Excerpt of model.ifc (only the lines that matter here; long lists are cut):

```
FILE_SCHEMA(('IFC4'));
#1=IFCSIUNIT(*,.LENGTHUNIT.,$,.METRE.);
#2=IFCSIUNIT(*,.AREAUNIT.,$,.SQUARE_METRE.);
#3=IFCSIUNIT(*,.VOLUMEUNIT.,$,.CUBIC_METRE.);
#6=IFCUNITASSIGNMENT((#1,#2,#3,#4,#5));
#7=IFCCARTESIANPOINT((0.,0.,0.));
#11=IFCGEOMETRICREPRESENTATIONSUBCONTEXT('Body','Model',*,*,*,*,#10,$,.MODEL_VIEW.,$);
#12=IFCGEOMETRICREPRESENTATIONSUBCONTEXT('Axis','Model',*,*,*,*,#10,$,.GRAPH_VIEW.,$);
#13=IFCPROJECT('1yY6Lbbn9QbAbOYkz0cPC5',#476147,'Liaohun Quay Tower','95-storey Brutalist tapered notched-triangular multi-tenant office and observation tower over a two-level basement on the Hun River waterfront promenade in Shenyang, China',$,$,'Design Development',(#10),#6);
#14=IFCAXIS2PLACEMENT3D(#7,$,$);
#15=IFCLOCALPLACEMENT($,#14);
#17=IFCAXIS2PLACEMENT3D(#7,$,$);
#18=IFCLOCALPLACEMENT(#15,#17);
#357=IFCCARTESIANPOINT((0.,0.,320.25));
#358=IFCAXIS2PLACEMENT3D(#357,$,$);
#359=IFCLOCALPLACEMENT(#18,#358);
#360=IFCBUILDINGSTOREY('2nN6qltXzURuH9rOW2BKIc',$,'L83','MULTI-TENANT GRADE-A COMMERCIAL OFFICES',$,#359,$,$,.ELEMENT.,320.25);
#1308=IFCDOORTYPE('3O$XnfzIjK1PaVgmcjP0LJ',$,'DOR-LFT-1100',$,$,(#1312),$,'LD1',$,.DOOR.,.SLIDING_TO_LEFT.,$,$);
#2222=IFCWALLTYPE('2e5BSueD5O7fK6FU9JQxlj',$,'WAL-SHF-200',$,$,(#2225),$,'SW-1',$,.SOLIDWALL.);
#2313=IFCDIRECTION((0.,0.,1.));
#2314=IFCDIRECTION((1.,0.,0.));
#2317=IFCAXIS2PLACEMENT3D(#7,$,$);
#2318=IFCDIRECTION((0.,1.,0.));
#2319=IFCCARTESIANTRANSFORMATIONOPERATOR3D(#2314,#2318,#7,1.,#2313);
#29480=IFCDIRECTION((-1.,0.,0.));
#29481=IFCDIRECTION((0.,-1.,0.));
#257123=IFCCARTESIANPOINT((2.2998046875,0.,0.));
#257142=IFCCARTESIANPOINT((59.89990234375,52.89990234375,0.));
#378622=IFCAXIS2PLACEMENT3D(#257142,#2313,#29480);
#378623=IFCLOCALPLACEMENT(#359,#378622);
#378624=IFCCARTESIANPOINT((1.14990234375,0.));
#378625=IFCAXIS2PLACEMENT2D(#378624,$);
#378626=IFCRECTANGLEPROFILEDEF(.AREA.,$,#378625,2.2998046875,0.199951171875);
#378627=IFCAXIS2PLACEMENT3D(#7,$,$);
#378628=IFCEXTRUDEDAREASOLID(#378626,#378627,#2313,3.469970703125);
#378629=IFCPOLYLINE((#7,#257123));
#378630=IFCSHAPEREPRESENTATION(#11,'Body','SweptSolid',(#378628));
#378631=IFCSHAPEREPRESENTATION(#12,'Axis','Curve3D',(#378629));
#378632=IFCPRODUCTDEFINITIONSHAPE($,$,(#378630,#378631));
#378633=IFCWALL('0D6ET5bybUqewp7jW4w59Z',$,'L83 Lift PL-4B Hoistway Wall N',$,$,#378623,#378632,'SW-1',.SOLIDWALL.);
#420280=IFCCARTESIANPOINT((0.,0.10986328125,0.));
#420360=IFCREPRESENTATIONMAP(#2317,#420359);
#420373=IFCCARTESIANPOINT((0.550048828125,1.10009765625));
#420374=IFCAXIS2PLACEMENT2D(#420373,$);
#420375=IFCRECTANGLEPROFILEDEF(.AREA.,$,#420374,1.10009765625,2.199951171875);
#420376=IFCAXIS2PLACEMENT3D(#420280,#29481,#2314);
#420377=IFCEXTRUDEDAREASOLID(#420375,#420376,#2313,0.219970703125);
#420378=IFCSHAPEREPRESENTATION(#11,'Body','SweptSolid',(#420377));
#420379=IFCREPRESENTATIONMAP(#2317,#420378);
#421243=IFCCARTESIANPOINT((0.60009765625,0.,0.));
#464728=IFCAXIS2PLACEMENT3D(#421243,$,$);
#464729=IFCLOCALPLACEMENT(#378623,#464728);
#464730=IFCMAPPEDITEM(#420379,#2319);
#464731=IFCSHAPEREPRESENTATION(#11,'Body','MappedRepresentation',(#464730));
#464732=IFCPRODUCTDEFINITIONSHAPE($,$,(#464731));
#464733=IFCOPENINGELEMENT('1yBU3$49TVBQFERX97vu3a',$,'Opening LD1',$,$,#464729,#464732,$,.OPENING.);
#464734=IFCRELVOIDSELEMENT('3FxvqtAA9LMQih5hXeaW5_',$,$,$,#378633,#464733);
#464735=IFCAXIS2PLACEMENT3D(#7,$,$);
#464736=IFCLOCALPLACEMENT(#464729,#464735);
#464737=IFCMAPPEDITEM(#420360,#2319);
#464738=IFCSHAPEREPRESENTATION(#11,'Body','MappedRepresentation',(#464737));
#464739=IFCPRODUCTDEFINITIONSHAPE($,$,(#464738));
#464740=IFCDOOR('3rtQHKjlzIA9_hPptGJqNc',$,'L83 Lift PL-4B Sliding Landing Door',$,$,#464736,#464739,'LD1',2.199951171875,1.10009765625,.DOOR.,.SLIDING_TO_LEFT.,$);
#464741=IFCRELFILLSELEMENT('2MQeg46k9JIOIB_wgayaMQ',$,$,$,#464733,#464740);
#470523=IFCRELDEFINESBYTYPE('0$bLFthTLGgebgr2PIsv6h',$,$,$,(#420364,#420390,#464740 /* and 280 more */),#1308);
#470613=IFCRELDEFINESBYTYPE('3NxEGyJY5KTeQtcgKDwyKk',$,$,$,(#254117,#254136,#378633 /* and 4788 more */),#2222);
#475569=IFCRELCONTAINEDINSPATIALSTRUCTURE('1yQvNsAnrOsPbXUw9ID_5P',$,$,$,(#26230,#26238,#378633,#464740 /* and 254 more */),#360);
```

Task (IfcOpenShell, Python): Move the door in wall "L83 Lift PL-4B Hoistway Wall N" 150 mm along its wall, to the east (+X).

```python
import ifcopenshell
import ifcopenshell.api.geometry
import ifcopenshell.util.placement
import ifcopenshell.util.unit

model = ifcopenshell.open("model.ifc")
unit_scale = ifcopenshell.util.unit.calculate_unit_scale(model)

door = model.by_guid("3rtQHKjlzIA9_hPptGJqNc")
opening = door.FillsVoids[0].RelatingOpeningElement
wall = opening.VoidsElements[0].RelatingBuildingElement

wall_matrix = ifcopenshell.util.placement.get_local_placement(wall.ObjectPlacement)
shift = wall_matrix[:3, 0] * -0.15 / unit_scale
before = ifcopenshell.util.placement.get_local_placement(door.ObjectPlacement)[:3, 3].copy()

# The door is placed relative to its opening, so it follows when the opening moves.
matrix = ifcopenshell.util.placement.get_local_placement(opening.ObjectPlacement)
matrix[:3, 3] += shift
ifcopenshell.api.geometry.edit_object_placement(
    model, product=opening, matrix=matrix, is_si=False, should_transform_children=True
)

after = ifcopenshell.util.placement.get_local_placement(door.ObjectPlacement)[:3, 3]
print("door moved by", (after - before).round(3) + 0.0)

model.write("model-out.ifc")
```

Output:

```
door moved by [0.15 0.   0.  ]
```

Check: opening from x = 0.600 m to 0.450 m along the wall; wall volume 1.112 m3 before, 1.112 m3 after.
